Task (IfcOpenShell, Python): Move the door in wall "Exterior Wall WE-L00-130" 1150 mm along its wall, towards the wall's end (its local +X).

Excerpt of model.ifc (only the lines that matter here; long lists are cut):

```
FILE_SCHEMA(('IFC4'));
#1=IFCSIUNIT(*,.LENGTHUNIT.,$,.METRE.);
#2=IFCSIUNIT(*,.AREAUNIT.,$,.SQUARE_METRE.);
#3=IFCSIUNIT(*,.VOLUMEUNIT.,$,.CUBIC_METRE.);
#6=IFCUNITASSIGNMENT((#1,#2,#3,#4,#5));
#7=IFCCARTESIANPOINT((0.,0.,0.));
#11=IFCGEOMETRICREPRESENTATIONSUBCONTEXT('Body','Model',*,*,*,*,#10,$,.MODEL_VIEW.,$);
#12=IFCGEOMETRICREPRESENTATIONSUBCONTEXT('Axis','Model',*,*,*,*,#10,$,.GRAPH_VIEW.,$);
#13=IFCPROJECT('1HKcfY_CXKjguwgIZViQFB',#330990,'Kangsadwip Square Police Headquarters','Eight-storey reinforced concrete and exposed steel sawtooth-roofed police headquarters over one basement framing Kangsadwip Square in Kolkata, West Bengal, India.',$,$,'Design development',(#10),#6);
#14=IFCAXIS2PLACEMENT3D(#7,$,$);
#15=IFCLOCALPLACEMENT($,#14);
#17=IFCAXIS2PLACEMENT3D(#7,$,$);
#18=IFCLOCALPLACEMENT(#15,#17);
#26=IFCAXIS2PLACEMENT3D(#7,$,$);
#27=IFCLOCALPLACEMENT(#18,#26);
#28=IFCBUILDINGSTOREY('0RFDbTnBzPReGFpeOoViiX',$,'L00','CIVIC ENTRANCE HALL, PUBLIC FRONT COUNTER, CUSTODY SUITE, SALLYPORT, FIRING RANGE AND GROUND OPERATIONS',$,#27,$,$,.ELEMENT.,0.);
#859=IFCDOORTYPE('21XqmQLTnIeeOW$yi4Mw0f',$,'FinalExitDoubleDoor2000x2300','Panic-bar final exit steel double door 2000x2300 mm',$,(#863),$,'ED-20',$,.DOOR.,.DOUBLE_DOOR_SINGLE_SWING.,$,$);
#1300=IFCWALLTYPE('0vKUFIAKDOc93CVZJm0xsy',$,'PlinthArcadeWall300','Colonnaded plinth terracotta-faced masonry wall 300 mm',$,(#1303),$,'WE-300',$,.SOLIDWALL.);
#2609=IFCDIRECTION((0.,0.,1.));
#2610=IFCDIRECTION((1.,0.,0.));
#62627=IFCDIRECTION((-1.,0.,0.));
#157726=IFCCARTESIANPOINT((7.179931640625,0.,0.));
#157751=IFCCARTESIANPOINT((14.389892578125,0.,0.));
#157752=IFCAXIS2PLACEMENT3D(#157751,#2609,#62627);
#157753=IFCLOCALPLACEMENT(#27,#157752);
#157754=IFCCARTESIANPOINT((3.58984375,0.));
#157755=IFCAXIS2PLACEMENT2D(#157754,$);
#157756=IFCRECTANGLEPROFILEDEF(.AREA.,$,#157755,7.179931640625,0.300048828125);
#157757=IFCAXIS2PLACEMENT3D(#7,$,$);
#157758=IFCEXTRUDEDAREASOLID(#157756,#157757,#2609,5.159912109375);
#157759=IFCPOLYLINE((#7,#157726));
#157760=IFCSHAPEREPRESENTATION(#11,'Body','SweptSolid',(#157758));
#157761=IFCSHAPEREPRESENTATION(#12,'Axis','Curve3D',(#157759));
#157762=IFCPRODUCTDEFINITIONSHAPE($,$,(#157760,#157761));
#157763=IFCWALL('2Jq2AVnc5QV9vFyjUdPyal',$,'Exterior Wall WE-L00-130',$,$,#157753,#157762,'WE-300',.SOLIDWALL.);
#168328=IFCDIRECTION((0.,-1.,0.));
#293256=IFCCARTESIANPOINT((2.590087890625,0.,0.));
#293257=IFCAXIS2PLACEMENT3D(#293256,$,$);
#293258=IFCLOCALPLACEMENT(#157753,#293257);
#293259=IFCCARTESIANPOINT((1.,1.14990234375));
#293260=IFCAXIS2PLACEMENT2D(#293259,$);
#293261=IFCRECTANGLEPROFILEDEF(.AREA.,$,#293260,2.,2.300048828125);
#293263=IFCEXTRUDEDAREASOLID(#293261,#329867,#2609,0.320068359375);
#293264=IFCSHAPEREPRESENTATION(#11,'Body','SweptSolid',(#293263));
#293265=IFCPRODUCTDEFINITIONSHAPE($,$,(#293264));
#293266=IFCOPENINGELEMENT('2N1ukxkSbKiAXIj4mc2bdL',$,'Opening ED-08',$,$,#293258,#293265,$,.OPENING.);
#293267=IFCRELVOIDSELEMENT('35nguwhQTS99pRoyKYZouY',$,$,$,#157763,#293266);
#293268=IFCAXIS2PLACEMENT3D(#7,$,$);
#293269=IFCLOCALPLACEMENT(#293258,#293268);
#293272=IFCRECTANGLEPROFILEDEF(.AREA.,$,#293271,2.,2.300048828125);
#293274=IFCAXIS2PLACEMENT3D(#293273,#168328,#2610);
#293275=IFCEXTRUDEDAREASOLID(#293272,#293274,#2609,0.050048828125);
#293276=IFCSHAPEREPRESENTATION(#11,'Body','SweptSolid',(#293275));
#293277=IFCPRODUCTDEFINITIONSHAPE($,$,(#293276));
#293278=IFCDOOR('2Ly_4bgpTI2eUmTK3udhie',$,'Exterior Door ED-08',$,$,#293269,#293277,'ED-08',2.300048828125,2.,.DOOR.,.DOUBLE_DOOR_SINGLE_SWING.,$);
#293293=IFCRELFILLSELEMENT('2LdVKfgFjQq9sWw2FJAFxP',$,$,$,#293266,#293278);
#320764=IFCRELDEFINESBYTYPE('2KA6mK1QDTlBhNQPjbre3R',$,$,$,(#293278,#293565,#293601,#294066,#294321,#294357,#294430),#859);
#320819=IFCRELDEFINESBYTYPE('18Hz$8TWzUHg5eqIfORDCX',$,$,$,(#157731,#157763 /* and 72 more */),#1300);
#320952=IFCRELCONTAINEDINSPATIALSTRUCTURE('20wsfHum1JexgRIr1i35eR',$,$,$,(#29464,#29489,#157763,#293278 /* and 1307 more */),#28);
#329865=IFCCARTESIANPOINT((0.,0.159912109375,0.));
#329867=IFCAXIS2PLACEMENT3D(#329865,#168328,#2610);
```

```python
import ifcopenshell
import ifcopenshell.api.geometry
import ifcopenshell.util.placement
import ifcopenshell.util.unit

model = ifcopenshell.open("model.ifc")
unit_scale = ifcopenshell.util.unit.calculate_unit_scale(model)

door = model.by_guid("2Ly_4bgpTI2eUmTK3udhie")
opening = door.FillsVoids[0].RelatingOpeningElement
wall = opening.VoidsElements[0].RelatingBuildingElement

wall_matrix = ifcopenshell.util.placement.get_local_placement(wall.ObjectPlacement)
shift = wall_matrix[:3, 0] * 1.15 / unit_scale
before = ifcopenshell.util.placement.get_local_placement(door.ObjectPlacement)[:3, 3].copy()

# The door is placed relative to its opening, so it follows when the opening moves.
matrix = ifcopenshell.util.placement.get_local_placement(opening.ObjectPlacement)
matrix[:3, 3] += shift
ifcopenshell.api.geometry.edit_object_placement(
    model, product=opening, matrix=matrix, is_si=False, should_transform_children=True
)

after = ifcopenshell.util.placement.get_local_placement(door.ObjectPlacement)[:3, 3]
print("door moved by", (after - before).round(3) + 0.0)

model.write("model_rev.ifc")
```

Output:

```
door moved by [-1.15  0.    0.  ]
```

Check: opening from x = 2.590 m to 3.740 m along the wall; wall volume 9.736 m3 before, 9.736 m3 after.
